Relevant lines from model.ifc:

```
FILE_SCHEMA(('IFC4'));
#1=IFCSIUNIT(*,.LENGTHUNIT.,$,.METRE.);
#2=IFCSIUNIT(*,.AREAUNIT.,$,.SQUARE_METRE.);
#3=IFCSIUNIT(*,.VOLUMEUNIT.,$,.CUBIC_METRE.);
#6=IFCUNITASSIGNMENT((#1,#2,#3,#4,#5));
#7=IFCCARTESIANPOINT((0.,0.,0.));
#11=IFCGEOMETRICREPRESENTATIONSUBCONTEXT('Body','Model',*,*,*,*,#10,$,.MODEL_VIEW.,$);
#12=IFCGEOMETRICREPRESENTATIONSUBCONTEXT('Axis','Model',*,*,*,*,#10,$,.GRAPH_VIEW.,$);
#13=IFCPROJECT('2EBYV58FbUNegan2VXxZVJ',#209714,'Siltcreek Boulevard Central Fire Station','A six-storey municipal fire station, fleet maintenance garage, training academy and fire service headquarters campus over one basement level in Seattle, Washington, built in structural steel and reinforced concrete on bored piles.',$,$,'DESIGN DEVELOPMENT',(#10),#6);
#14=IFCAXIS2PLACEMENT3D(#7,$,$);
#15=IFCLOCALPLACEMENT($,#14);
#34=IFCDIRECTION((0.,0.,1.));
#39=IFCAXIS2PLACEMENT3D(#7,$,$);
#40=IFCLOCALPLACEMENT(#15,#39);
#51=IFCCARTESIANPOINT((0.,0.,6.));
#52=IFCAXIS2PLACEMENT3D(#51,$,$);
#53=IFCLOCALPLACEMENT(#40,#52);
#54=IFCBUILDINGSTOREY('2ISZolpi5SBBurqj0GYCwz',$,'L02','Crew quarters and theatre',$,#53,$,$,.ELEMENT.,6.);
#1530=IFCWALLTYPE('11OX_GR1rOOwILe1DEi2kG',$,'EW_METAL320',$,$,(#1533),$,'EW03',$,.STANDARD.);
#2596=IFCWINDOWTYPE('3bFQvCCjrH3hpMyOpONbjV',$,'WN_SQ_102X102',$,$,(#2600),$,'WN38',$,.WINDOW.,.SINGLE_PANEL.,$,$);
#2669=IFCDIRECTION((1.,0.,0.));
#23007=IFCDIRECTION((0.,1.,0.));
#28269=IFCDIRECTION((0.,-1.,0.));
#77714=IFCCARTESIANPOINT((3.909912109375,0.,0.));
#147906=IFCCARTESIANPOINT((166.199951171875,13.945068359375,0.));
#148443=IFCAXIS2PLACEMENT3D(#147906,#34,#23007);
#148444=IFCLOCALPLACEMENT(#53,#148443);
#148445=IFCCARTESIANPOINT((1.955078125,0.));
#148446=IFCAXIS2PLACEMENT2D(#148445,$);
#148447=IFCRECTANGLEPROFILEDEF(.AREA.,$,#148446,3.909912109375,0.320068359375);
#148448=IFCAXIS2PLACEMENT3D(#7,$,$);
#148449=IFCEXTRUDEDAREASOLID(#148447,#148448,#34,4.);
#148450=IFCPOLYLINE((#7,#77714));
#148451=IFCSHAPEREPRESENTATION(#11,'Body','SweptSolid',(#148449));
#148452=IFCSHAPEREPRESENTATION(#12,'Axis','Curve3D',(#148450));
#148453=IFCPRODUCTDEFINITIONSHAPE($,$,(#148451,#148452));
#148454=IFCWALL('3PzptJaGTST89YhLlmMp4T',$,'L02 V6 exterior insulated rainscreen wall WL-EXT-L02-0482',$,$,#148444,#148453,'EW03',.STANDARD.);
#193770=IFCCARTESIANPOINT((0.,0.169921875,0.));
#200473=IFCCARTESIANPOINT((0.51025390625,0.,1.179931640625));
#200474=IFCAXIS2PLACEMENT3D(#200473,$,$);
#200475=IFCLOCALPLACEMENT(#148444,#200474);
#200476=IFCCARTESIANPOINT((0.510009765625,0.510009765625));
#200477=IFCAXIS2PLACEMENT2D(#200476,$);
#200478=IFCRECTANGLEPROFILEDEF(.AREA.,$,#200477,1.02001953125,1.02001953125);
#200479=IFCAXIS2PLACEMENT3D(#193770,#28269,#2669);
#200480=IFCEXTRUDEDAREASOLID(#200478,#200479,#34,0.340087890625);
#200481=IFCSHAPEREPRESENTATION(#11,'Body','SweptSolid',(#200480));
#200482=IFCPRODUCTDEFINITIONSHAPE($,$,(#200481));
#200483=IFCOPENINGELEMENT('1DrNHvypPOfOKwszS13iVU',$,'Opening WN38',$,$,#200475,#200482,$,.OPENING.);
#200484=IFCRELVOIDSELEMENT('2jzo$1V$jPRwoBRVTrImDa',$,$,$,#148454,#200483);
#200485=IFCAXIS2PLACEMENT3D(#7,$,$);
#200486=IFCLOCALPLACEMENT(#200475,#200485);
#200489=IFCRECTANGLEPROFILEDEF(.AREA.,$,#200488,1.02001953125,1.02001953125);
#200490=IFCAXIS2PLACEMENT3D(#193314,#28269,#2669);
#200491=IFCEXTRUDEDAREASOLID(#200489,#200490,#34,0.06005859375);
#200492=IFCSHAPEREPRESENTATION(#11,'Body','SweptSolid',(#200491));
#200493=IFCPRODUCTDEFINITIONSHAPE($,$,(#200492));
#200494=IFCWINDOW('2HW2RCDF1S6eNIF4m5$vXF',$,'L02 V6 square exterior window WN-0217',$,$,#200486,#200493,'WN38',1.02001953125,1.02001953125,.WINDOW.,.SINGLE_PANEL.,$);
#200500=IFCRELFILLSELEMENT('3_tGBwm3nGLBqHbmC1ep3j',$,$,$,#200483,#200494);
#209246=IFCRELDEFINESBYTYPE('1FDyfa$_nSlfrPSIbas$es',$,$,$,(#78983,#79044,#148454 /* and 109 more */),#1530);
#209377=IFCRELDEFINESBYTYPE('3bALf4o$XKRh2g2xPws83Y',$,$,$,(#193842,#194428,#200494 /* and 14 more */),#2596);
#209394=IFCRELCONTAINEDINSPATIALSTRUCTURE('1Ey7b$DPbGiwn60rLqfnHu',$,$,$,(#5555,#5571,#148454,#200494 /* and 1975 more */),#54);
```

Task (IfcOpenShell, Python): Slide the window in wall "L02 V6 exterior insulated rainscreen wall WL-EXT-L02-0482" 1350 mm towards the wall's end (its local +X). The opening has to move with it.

```python
import ifcopenshell
import ifcopenshell.api.geometry
import ifcopenshell.util.placement

model = ifcopenshell.open("model.ifc")

window = model.by_guid("2HW2RCDF1S6eNIF4m5$vXF")
opening = window.FillsVoids[0].RelatingOpeningElement
wall = opening.VoidsElements[0].RelatingBuildingElement

wall_matrix = ifcopenshell.util.placement.get_local_placement(wall.ObjectPlacement)
shift = wall_matrix[:3, 0] * 1.35
before = ifcopenshell.util.placement.get_local_placement(window.ObjectPlacement)[:3, 3].copy()

# The window is placed relative to its opening, so it follows when the opening moves.
matrix = ifcopenshell.util.placement.get_local_placement(opening.ObjectPlacement)
matrix[:3, 3] += shift
ifcopenshell.api.geometry.edit_object_placement(
    model, product=opening, matrix=matrix, is_si=False, should_transform_children=True
)

after = ifcopenshell.util.placement.get_local_placement(window.ObjectPlacement)[:3, 3]
print("window moved by", (after - before).round(3) + 0.0)

model.write("model-out.ifc")
```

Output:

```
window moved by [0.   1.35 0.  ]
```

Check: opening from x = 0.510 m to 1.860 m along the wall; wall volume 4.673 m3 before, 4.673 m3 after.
